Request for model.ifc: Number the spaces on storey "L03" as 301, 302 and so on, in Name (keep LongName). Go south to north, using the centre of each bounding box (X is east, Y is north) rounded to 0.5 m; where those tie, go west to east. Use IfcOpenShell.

First a look at what the model holds.

```python
import ifcopenshell
import ifcopenshell.util.element
import ifcopenshell.util.placement

model = ifcopenshell.open("model.ifc")
print(model.schema)
storey = next(s for s in model.by_type("IfcBuildingStorey") if s.Name == "L03")
spaces = [e for e in ifcopenshell.util.element.get_decomposition(storey) if e.is_a("IfcSpace")]
for e in sorted(spaces, key=lambda e: e.id()):
    origin = ifcopenshell.util.placement.get_local_placement(e.ObjectPlacement)[:3, 3]
    print(e.id(), e.Name, e.LongName, origin.round(2) + 0.0, sep=" | ")
```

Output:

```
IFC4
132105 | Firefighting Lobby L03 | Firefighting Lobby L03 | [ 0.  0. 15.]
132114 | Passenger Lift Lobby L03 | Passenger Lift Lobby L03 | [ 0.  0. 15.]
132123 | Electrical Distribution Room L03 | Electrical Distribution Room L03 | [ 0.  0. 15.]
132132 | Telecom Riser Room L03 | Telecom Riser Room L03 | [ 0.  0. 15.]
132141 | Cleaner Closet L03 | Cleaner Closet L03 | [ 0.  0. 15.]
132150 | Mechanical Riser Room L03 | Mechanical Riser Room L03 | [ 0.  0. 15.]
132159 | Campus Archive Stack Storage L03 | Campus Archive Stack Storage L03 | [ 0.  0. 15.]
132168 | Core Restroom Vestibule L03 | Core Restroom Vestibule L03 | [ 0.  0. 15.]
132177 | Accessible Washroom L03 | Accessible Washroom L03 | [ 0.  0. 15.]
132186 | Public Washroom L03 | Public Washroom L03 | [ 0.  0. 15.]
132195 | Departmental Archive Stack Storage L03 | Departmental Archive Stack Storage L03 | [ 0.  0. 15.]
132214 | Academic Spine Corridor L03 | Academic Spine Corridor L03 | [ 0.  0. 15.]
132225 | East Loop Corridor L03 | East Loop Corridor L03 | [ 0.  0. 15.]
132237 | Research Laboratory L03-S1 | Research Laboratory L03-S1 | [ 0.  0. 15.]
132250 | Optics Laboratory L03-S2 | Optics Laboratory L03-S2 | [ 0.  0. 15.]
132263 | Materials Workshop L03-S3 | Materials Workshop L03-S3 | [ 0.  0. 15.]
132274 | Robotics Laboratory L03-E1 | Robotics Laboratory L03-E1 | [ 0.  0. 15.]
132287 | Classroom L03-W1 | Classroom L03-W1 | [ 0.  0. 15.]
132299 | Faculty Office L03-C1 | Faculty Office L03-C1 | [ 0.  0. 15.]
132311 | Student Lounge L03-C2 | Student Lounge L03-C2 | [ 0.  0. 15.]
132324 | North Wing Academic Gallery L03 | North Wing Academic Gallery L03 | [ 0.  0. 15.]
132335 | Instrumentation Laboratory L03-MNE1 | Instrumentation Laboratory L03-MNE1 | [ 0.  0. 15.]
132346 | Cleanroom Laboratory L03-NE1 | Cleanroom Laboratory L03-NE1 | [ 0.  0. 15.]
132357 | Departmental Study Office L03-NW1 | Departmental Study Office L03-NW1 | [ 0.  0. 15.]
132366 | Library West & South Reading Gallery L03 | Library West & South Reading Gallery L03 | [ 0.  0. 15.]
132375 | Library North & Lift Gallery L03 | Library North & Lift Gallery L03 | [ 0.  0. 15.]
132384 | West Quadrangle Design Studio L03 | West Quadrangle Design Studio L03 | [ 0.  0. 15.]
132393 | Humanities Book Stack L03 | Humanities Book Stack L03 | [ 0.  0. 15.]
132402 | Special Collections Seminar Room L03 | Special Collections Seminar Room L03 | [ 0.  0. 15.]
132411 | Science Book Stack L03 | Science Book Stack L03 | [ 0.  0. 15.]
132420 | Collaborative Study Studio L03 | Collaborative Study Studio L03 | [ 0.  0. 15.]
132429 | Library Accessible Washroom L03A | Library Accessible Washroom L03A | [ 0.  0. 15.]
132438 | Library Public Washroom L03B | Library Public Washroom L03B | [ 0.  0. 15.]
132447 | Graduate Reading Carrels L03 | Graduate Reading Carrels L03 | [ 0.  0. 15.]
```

```python
import ifcopenshell
import ifcopenshell.geom
import ifcopenshell.util.element
import ifcopenshell.util.shape

model = ifcopenshell.open("model.ifc")
settings = ifcopenshell.geom.settings()
settings.set("use-world-coords", True)


def centre(element):
    shape = ifcopenshell.geom.create_shape(settings, element)
    return ifcopenshell.util.shape.get_bbox_centroid(shape.geometry)


storey = next(s for s in model.by_type("IfcBuildingStorey") if s.Name == "L03")
spaces = [e for e in ifcopenshell.util.element.get_decomposition(storey) if e.is_a("IfcSpace")]

# Insertion points can sit at a corner or the storey origin, so sort by the geometry (in metres).
centres = {e: centre(e) for e in spaces}
spaces.sort(key=lambda e: (round(centres[e][1] / 0.5), centres[e][0]))

for i, e in enumerate(spaces, start=1):
    number = f"3{i:02d}"
    e.Name = number
    print(e.id(), number)

model.write("model_rev.ifc")
```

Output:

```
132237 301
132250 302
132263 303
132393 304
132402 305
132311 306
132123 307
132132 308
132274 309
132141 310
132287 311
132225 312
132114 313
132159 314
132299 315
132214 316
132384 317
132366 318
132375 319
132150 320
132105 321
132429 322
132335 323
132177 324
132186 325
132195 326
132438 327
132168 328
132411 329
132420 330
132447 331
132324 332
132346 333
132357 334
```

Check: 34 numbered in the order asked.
